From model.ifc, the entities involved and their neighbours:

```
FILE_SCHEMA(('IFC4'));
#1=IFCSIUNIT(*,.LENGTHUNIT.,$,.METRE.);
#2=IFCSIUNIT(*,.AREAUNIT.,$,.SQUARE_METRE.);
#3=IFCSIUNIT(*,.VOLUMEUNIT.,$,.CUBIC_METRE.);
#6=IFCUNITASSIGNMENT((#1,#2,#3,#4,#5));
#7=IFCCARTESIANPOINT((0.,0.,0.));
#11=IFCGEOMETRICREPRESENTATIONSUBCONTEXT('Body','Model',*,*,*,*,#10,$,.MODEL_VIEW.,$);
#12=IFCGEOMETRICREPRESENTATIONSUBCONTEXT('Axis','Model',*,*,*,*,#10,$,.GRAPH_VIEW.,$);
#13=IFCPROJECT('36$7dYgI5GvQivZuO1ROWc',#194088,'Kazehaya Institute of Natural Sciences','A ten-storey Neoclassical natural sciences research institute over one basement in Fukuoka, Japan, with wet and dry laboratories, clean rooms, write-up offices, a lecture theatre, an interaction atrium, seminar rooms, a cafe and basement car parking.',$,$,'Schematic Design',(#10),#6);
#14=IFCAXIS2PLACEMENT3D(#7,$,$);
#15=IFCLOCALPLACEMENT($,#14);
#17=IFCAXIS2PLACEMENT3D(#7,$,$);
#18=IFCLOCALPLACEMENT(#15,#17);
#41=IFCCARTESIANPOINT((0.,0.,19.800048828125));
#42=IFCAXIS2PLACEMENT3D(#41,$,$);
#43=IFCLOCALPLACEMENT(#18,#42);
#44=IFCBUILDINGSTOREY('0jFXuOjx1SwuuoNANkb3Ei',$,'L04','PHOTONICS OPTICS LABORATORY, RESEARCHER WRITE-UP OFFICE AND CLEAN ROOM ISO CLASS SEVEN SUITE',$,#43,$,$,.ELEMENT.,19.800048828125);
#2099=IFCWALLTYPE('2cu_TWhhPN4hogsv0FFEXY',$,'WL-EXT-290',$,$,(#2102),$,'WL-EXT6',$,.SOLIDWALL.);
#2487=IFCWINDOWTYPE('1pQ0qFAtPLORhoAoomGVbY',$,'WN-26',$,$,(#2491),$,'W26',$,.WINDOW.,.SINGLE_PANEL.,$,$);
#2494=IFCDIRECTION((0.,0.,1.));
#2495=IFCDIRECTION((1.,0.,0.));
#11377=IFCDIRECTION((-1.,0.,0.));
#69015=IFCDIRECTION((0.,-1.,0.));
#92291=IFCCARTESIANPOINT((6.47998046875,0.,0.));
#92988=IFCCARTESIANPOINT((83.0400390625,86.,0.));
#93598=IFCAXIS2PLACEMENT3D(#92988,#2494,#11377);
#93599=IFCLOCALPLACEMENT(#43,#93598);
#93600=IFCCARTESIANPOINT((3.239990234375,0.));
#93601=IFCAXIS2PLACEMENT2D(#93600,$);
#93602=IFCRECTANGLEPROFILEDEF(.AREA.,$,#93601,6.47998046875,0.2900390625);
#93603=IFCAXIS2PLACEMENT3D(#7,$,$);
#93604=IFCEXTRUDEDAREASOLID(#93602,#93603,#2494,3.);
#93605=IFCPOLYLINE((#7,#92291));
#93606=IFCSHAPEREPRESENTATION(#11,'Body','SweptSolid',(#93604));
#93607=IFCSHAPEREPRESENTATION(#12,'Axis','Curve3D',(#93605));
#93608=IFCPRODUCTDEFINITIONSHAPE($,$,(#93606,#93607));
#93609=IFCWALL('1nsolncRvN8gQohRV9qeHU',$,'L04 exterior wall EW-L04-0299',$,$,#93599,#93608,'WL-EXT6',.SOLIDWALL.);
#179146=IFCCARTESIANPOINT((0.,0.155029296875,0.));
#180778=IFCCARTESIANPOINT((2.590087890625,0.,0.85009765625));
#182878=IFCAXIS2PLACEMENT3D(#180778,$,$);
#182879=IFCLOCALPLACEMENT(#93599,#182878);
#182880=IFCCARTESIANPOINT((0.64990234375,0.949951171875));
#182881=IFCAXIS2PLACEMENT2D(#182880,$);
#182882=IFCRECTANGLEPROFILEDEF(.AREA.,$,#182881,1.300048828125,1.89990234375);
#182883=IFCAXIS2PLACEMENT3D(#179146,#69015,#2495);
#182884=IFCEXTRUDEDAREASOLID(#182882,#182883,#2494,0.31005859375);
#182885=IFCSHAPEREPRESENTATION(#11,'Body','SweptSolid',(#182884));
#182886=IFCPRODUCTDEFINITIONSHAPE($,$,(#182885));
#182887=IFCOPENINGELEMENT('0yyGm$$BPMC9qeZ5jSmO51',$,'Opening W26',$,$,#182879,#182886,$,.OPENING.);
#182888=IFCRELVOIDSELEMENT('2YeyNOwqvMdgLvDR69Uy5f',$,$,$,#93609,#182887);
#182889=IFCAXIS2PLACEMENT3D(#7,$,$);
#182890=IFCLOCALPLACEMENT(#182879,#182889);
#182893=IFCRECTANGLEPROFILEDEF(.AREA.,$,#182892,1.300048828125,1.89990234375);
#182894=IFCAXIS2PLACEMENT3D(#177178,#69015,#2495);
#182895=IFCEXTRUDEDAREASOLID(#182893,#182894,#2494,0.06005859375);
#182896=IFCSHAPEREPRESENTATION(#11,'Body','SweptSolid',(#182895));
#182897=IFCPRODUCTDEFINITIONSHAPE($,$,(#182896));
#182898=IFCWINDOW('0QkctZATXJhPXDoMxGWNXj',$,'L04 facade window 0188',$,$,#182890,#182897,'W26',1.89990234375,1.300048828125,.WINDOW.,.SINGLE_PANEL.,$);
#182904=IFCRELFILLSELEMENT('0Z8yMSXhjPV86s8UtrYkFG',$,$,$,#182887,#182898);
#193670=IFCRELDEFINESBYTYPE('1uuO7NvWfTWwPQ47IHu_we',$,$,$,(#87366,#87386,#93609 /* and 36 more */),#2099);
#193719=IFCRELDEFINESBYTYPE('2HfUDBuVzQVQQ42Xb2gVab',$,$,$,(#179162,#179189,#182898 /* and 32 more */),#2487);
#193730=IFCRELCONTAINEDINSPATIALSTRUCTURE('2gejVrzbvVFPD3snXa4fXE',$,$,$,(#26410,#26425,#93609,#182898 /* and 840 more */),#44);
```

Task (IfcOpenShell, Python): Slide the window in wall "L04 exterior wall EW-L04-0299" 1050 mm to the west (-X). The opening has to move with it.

```python
import ifcopenshell
import ifcopenshell.api.geometry
import ifcopenshell.util.placement
import ifcopenshell.util.unit

model = ifcopenshell.open("model.ifc")
unit_scale = ifcopenshell.util.unit.calculate_unit_scale(model)

window = model.by_guid("0QkctZATXJhPXDoMxGWNXj")
opening = window.FillsVoids[0].RelatingOpeningElement
wall = opening.VoidsElements[0].RelatingBuildingElement

wall_matrix = ifcopenshell.util.placement.get_local_placement(wall.ObjectPlacement)
shift = wall_matrix[:3, 0] * 1.05 / unit_scale
before = ifcopenshell.util.placement.get_local_placement(window.ObjectPlacement)[:3, 3].copy()

# The window is placed relative to its opening, so it follows when the opening moves.
matrix = ifcopenshell.util.placement.get_local_placement(opening.ObjectPlacement)
matrix[:3, 3] += shift
ifcopenshell.api.geometry.edit_object_placement(
    model, product=opening, matrix=matrix, is_si=False, should_transform_children=True
)

after = ifcopenshell.util.placement.get_local_placement(window.ObjectPlacement)[:3, 3]
print("window moved by", (after - before).round(3) + 0.0)

model.write("model_updated.ifc")
```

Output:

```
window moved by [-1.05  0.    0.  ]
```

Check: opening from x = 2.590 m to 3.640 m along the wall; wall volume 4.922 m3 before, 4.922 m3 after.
